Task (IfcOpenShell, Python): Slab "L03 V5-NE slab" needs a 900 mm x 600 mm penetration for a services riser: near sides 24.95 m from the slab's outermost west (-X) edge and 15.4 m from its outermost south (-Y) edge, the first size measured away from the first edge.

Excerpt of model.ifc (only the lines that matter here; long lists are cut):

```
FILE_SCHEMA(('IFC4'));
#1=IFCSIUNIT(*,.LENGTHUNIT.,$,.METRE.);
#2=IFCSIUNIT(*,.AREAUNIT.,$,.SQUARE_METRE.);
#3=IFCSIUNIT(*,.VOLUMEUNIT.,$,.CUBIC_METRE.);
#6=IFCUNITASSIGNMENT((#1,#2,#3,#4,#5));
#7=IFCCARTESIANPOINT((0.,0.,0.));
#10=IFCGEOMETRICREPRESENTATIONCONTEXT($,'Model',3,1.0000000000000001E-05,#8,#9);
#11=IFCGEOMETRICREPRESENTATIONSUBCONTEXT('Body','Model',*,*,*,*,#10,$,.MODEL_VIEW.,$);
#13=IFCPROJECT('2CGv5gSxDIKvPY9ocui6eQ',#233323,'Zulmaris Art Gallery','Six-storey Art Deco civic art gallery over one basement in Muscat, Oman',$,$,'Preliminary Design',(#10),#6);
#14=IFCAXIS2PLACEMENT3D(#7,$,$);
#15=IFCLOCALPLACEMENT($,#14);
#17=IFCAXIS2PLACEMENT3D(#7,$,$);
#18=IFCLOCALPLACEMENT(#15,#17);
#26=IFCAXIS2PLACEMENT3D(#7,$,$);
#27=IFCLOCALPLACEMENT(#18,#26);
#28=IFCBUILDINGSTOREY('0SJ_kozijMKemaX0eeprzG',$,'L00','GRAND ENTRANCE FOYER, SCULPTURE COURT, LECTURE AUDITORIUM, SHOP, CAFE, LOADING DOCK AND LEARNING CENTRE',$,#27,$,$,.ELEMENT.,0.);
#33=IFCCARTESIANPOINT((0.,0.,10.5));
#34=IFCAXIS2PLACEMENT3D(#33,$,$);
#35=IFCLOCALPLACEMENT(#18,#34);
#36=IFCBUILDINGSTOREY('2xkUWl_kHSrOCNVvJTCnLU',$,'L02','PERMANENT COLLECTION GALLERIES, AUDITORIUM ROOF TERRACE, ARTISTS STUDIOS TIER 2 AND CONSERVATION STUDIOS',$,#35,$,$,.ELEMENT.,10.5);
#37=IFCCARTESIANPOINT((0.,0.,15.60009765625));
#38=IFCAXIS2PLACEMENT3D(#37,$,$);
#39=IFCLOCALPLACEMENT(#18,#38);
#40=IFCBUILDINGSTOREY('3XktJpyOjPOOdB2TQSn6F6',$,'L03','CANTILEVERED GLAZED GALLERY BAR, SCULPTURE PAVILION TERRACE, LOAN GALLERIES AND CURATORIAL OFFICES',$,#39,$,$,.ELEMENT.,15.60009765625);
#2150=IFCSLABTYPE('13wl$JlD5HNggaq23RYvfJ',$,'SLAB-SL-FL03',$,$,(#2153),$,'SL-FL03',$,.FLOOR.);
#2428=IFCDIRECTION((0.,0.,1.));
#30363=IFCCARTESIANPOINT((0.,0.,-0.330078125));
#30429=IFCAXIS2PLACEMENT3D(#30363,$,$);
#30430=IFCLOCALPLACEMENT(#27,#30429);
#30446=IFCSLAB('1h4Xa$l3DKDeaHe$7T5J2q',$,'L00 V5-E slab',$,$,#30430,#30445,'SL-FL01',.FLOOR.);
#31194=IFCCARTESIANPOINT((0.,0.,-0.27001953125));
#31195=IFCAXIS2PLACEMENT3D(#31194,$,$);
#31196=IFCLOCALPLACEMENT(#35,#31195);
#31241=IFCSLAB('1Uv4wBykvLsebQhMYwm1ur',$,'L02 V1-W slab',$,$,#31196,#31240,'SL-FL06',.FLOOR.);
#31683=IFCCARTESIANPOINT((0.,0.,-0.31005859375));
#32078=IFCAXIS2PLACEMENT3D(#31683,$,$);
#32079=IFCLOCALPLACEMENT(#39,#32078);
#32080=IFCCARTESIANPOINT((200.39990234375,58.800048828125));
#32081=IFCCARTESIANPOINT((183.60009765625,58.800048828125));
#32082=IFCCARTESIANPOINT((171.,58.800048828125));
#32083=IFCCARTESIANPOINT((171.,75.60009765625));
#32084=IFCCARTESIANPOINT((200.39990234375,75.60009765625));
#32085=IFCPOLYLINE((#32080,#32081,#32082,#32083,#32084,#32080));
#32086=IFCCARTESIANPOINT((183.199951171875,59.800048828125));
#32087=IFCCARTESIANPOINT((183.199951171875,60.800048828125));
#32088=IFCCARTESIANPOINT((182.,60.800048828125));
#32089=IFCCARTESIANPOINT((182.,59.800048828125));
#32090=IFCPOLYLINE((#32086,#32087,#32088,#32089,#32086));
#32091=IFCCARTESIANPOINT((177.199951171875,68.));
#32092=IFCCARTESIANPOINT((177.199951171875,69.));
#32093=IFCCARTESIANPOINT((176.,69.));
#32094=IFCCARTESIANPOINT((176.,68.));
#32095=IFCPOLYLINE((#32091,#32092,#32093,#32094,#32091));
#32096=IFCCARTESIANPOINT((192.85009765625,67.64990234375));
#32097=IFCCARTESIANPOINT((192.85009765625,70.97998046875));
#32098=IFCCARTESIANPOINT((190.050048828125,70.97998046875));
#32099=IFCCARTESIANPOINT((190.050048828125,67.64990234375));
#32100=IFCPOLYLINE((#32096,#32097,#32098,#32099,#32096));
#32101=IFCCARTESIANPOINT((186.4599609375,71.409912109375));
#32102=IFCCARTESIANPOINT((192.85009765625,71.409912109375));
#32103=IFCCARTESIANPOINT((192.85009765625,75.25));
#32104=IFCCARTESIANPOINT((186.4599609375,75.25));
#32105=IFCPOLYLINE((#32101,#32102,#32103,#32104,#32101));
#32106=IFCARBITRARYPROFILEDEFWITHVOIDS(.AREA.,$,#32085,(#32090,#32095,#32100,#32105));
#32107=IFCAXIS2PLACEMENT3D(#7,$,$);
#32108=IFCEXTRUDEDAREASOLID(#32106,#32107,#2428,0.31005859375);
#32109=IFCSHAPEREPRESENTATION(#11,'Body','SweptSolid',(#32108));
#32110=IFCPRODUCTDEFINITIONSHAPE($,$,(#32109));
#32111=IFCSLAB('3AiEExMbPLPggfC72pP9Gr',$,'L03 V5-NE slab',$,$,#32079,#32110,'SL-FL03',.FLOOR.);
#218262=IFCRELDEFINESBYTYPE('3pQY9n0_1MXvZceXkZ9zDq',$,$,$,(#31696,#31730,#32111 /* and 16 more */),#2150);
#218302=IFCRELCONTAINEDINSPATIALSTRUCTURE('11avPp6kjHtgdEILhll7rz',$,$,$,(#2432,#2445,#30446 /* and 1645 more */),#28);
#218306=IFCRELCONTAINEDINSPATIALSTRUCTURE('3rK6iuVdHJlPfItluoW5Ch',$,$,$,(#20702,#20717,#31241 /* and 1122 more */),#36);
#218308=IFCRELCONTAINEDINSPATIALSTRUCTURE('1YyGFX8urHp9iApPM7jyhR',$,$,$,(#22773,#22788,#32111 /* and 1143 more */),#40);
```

```python
import numpy as np
import ifcopenshell
import ifcopenshell.api.feature
import ifcopenshell.api.geometry
import ifcopenshell.api.root
import ifcopenshell.geom
import ifcopenshell.util.placement
import ifcopenshell.util.representation
import ifcopenshell.util.shape
import ifcopenshell.util.unit

model = ifcopenshell.open("model.ifc")
unit_scale = ifcopenshell.util.unit.calculate_unit_scale(model)
settings = ifcopenshell.geom.settings()


def volume(element):
    """Net volume in cubic metres, openings subtracted."""
    shape = ifcopenshell.geom.create_shape(settings, element)
    return ifcopenshell.util.shape.get_volume(shape.geometry)


slab = model.by_id(32111)
before = volume(slab)

# Extent in the slab's own axes, in metres. The edges named are its -X and -Y sides.
slab_shape = ifcopenshell.geom.create_shape(settings, slab)
vertices = ifcopenshell.util.shape.get_vertices(slab_shape.geometry)
x_min, y_min, bottom = vertices.min(axis=0)
top = vertices[:, 2].max()

opening = ifcopenshell.api.root.create_entity(model, ifc_class="IfcOpeningElement", name="Services riser opening", predefined_type="OPENING")
context = ifcopenshell.util.representation.get_context(model, "Model", "Body", "MODEL_VIEW")
width, depth = 0.9, 0.6
outline = [(0.0, 0.0), (width, 0.0), (width, depth), (0.0, depth), (0.0, 0.0)]
# Overshoot both faces by 50 mm so the cut is clean.
shape = ifcopenshell.api.geometry.add_slab_representation(
    model, context=context, depth=top - bottom + 0.1, polyline=outline
)
ifcopenshell.api.geometry.assign_representation(model, product=opening, representation=shape)

matrix = ifcopenshell.util.placement.get_local_placement(slab.ObjectPlacement)
matrix[:, 3] = matrix @ np.append(np.array([x_min + 24.95, y_min + 15.4, bottom - 0.05]) / unit_scale, 1.0)
ifcopenshell.api.geometry.edit_object_placement(model, product=opening, matrix=matrix, is_si=False)
ifcopenshell.api.feature.add_feature(model, feature=opening, element=slab)

after = volume(slab)

print(f"slab volume {before:.3f} -> {after:.3f} m3")

model.write("model_updated.ifc")
```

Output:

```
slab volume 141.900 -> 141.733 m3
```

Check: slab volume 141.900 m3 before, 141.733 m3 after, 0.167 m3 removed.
